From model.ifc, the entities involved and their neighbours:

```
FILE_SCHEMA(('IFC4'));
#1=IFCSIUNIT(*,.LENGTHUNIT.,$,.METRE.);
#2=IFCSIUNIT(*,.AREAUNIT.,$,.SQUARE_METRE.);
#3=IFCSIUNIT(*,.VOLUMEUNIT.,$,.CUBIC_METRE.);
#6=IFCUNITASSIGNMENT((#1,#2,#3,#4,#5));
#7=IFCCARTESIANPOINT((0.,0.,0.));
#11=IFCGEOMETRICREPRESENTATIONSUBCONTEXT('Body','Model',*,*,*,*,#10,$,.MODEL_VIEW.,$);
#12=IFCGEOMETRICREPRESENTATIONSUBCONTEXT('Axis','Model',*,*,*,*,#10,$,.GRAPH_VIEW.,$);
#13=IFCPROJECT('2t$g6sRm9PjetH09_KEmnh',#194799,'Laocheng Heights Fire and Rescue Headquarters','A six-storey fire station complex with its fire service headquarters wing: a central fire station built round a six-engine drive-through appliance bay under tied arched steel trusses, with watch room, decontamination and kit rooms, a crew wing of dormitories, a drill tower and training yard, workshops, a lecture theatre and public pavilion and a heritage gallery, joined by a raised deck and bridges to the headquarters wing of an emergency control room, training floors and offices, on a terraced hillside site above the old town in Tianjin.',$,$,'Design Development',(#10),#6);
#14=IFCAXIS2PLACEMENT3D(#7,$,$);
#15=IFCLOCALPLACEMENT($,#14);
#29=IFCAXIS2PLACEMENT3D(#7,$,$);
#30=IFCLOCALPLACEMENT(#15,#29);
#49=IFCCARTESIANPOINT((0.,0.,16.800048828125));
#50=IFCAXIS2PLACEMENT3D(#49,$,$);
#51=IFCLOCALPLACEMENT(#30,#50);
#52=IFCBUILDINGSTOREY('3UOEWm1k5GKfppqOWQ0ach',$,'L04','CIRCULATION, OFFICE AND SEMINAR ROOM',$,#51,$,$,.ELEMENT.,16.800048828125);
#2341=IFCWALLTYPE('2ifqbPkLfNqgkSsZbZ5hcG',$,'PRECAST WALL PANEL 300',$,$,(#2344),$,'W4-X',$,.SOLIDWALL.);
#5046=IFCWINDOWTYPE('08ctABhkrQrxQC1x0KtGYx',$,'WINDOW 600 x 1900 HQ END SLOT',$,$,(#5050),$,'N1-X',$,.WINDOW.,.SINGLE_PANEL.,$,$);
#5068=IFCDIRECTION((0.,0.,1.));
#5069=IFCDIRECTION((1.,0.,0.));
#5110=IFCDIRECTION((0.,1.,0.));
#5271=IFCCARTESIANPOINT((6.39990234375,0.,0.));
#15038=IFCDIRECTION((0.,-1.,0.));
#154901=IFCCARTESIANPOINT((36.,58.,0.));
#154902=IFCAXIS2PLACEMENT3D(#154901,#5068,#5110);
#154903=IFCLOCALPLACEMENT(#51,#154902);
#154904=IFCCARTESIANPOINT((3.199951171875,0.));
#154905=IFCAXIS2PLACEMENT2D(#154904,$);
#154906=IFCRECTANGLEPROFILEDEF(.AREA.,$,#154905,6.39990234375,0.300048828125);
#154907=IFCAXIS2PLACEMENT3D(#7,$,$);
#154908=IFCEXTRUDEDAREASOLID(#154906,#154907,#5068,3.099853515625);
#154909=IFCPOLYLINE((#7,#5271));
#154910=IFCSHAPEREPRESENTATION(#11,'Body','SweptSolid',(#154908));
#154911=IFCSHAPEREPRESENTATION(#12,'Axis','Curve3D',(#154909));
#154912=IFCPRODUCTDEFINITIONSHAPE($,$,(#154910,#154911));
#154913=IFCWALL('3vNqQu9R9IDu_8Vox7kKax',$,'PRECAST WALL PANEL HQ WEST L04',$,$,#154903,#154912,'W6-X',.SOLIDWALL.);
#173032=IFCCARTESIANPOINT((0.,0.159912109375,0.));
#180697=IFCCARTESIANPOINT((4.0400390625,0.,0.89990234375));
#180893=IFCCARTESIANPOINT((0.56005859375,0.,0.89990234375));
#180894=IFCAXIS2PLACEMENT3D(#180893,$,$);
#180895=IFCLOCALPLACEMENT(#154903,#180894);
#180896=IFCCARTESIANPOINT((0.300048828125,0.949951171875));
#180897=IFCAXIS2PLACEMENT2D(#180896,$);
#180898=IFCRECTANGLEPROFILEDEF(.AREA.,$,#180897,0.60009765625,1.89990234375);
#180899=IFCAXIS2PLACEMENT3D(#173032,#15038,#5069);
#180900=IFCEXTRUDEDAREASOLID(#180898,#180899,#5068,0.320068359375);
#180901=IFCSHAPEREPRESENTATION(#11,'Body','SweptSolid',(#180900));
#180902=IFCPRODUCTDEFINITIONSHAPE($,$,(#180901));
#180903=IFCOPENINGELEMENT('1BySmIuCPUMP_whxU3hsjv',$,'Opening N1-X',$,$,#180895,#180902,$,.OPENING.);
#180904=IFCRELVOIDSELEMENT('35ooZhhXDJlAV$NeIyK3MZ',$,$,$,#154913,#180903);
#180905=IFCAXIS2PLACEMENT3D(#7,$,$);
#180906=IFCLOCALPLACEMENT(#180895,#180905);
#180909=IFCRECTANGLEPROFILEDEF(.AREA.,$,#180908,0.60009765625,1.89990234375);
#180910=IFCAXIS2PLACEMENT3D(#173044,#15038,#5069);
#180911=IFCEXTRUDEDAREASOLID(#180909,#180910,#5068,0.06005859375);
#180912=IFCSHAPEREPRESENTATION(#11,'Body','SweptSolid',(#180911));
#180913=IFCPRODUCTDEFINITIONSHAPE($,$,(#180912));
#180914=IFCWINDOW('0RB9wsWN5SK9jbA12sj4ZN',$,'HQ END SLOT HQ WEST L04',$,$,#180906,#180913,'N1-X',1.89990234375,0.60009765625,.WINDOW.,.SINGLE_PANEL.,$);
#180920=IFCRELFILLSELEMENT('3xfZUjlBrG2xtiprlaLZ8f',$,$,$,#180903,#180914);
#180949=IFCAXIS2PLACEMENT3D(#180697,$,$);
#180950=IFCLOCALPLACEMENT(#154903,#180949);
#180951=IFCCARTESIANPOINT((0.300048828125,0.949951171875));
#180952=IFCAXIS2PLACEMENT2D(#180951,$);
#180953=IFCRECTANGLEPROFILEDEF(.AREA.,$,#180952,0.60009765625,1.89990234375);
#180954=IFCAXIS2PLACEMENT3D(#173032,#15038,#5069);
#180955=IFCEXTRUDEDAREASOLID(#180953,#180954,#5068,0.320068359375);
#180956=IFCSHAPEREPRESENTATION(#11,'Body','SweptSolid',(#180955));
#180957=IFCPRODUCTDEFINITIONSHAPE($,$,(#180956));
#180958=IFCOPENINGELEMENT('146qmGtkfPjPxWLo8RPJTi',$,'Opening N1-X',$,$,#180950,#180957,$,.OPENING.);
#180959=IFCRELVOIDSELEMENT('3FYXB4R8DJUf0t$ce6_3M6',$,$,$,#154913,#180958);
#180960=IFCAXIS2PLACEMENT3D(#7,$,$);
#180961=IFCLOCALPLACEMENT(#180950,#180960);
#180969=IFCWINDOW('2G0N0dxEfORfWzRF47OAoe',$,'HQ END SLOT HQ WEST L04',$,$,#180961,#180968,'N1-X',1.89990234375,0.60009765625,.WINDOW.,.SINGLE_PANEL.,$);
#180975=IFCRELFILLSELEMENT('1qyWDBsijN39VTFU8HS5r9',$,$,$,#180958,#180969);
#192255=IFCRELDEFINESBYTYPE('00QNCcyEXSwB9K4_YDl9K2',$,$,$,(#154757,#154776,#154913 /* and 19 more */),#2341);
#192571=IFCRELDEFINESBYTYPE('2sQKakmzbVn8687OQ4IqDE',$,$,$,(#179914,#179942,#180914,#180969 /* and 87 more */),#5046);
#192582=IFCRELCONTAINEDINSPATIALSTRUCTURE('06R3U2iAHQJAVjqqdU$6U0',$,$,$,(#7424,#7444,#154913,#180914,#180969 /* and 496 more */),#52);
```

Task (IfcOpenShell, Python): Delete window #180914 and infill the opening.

```python
import ifcopenshell
import ifcopenshell.api.feature
import ifcopenshell.api.root
import ifcopenshell.geom
import ifcopenshell.util.shape

model = ifcopenshell.open("model.ifc")
settings = ifcopenshell.geom.settings()


def volume(element):
    """Net volume in cubic metres, openings subtracted."""
    shape = ifcopenshell.geom.create_shape(settings, element)
    return ifcopenshell.util.shape.get_volume(shape.geometry)


window = model.by_id(180914)
opening = window.FillsVoids[0].RelatingOpeningElement
wall = opening.VoidsElements[0].RelatingBuildingElement
before = volume(wall)

ifcopenshell.api.root.remove_product(model, product=window)
ifcopenshell.api.feature.remove_feature(model, feature=opening)

after = volume(wall)

print(f"wall volume {before:.3f} -> {after:.3f} m3")

model.write("model-out.ifc")
```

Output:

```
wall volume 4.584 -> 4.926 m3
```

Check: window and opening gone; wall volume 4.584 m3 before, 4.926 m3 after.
